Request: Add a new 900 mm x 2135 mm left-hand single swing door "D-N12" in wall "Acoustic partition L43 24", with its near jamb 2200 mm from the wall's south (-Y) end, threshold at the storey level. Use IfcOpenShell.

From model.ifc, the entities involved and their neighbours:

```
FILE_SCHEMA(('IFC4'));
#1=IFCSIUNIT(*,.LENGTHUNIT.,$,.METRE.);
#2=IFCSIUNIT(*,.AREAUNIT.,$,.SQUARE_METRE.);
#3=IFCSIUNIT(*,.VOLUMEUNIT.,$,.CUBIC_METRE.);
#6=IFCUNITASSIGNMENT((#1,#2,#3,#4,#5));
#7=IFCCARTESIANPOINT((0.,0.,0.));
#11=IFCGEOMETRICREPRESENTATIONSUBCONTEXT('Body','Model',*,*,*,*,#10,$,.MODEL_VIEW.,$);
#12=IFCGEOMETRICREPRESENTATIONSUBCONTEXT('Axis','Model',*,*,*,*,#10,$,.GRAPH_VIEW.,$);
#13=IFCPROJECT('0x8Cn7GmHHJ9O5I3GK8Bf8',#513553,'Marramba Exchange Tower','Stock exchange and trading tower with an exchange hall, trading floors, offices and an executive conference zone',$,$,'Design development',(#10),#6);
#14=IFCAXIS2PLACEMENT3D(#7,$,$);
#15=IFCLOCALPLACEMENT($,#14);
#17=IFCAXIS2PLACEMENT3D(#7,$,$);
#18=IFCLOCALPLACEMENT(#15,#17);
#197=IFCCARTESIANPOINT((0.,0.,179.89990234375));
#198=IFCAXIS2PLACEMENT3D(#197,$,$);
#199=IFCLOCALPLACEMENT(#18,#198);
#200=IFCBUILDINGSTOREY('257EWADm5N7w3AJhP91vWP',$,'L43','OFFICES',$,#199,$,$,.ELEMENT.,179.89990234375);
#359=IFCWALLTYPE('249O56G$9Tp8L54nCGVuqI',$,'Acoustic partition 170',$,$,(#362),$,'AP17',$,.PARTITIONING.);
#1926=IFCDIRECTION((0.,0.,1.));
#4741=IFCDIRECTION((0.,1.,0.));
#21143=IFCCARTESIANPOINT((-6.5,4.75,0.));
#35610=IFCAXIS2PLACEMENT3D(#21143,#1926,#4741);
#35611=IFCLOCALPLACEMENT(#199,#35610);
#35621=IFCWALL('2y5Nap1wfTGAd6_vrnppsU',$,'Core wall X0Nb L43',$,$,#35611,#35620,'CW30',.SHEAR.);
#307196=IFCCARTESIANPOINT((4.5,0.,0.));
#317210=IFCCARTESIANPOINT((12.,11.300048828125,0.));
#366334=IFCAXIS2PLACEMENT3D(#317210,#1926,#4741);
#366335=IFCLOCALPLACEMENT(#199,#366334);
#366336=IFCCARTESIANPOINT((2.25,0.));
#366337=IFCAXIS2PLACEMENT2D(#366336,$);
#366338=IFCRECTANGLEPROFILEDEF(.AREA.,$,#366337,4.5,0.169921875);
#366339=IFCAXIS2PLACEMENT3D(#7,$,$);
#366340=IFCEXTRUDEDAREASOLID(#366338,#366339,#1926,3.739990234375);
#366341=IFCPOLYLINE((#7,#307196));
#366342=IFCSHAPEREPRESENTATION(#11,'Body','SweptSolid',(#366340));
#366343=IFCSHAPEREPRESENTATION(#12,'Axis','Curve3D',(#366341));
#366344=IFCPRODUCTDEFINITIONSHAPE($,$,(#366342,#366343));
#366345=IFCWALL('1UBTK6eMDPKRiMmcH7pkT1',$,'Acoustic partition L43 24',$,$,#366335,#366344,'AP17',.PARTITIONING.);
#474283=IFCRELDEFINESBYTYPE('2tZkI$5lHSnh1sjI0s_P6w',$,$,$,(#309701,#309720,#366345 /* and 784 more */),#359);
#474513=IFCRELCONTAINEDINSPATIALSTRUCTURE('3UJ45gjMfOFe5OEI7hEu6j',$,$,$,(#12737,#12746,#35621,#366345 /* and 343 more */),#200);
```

```python
import numpy as np
import ifcopenshell
import ifcopenshell.api.feature
import ifcopenshell.api.geometry
import ifcopenshell.api.root
import ifcopenshell.api.spatial
import ifcopenshell.geom
import ifcopenshell.util.element
import ifcopenshell.util.placement
import ifcopenshell.util.representation
import ifcopenshell.util.shape
import ifcopenshell.util.unit

model = ifcopenshell.open("model.ifc")
unit_scale = ifcopenshell.util.unit.calculate_unit_scale(model)
settings = ifcopenshell.geom.settings()


def volume(element):
    """Net volume in cubic metres, openings subtracted."""
    shape = ifcopenshell.geom.create_shape(settings, element)
    return ifcopenshell.util.shape.get_volume(shape.geometry)


wall = model.by_guid("1UBTK6eMDPKRiMmcH7pkT1")
storey = ifcopenshell.util.element.get_container(wall, ifc_class="IfcBuildingStorey")
context = ifcopenshell.util.representation.get_context(model, "Model", "Body", "MODEL_VIEW")
before = volume(wall)

width, height, from_end, sill = 0.9, 2.135, 2.2, 0.0  # metres

# The wall runs along its own X axis, and the end named is its -X end.
wall_shape = ifcopenshell.geom.create_shape(settings, wall)
x, y, z = ifcopenshell.util.shape.get_vertices(wall_shape.geometry).T
start = x.min() + from_end
face, thickness = float(y.min()), float(y.max() - y.min())
wall_matrix = ifcopenshell.util.placement.get_local_placement(wall.ObjectPlacement)
level = ifcopenshell.util.placement.get_local_placement(storey.ObjectPlacement)[2, 3]


def in_wall(x, y):
    """Placement at x, y metres in the wall's axes, at sill height."""
    matrix = wall_matrix.copy()
    matrix[:, 3] = wall_matrix @ np.array([x / unit_scale, y / unit_scale, 0.0, 1.0])
    matrix[2, 3] = level + sill / unit_scale
    return matrix


# Opening: a box that overshoots both wall faces by 50 mm.
opening = ifcopenshell.api.root.create_entity(model, ifc_class="IfcOpeningElement", predefined_type="OPENING")
box = ifcopenshell.api.geometry.add_wall_representation(
    model, context=context, length=width, height=height, thickness=thickness + 0.1
)
ifcopenshell.api.geometry.assign_representation(model, product=opening, representation=box)
ifcopenshell.api.geometry.edit_object_placement(model, product=opening, matrix=in_wall(start, face - 0.05), is_si=False)
ifcopenshell.api.feature.add_feature(model, feature=opening, element=wall)

door = ifcopenshell.api.root.create_entity(model, ifc_class="IfcDoor", name="D-N12", predefined_type="DOOR")
door.OverallWidth, door.OverallHeight = width / unit_scale, height / unit_scale
door.OperationType = "SINGLE_SWING_LEFT"
body = ifcopenshell.api.geometry.add_door_representation(
    model,
    context=context,
    overall_width=door.OverallWidth,
    overall_height=door.OverallHeight,
    operation_type="SINGLE_SWING_LEFT",
    lining_properties={"LiningDepth": thickness / unit_scale, "ThresholdDepth": thickness / unit_scale},
)
ifcopenshell.api.geometry.assign_representation(model, product=door, representation=body)
ifcopenshell.api.spatial.assign_container(model, products=[door], relating_structure=storey)
ifcopenshell.api.feature.add_filling(model, opening=opening, element=door)

# The lining spans the wall, so the door starts at the wall face.
ifcopenshell.api.geometry.edit_object_placement(model, product=door, matrix=in_wall(start, face), is_si=False)

after = volume(wall)

print(f"wall volume {before:.3f} -> {after:.3f} m3")

model.write("model-out.ifc")
```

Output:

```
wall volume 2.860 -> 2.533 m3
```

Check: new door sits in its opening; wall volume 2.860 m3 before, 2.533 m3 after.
